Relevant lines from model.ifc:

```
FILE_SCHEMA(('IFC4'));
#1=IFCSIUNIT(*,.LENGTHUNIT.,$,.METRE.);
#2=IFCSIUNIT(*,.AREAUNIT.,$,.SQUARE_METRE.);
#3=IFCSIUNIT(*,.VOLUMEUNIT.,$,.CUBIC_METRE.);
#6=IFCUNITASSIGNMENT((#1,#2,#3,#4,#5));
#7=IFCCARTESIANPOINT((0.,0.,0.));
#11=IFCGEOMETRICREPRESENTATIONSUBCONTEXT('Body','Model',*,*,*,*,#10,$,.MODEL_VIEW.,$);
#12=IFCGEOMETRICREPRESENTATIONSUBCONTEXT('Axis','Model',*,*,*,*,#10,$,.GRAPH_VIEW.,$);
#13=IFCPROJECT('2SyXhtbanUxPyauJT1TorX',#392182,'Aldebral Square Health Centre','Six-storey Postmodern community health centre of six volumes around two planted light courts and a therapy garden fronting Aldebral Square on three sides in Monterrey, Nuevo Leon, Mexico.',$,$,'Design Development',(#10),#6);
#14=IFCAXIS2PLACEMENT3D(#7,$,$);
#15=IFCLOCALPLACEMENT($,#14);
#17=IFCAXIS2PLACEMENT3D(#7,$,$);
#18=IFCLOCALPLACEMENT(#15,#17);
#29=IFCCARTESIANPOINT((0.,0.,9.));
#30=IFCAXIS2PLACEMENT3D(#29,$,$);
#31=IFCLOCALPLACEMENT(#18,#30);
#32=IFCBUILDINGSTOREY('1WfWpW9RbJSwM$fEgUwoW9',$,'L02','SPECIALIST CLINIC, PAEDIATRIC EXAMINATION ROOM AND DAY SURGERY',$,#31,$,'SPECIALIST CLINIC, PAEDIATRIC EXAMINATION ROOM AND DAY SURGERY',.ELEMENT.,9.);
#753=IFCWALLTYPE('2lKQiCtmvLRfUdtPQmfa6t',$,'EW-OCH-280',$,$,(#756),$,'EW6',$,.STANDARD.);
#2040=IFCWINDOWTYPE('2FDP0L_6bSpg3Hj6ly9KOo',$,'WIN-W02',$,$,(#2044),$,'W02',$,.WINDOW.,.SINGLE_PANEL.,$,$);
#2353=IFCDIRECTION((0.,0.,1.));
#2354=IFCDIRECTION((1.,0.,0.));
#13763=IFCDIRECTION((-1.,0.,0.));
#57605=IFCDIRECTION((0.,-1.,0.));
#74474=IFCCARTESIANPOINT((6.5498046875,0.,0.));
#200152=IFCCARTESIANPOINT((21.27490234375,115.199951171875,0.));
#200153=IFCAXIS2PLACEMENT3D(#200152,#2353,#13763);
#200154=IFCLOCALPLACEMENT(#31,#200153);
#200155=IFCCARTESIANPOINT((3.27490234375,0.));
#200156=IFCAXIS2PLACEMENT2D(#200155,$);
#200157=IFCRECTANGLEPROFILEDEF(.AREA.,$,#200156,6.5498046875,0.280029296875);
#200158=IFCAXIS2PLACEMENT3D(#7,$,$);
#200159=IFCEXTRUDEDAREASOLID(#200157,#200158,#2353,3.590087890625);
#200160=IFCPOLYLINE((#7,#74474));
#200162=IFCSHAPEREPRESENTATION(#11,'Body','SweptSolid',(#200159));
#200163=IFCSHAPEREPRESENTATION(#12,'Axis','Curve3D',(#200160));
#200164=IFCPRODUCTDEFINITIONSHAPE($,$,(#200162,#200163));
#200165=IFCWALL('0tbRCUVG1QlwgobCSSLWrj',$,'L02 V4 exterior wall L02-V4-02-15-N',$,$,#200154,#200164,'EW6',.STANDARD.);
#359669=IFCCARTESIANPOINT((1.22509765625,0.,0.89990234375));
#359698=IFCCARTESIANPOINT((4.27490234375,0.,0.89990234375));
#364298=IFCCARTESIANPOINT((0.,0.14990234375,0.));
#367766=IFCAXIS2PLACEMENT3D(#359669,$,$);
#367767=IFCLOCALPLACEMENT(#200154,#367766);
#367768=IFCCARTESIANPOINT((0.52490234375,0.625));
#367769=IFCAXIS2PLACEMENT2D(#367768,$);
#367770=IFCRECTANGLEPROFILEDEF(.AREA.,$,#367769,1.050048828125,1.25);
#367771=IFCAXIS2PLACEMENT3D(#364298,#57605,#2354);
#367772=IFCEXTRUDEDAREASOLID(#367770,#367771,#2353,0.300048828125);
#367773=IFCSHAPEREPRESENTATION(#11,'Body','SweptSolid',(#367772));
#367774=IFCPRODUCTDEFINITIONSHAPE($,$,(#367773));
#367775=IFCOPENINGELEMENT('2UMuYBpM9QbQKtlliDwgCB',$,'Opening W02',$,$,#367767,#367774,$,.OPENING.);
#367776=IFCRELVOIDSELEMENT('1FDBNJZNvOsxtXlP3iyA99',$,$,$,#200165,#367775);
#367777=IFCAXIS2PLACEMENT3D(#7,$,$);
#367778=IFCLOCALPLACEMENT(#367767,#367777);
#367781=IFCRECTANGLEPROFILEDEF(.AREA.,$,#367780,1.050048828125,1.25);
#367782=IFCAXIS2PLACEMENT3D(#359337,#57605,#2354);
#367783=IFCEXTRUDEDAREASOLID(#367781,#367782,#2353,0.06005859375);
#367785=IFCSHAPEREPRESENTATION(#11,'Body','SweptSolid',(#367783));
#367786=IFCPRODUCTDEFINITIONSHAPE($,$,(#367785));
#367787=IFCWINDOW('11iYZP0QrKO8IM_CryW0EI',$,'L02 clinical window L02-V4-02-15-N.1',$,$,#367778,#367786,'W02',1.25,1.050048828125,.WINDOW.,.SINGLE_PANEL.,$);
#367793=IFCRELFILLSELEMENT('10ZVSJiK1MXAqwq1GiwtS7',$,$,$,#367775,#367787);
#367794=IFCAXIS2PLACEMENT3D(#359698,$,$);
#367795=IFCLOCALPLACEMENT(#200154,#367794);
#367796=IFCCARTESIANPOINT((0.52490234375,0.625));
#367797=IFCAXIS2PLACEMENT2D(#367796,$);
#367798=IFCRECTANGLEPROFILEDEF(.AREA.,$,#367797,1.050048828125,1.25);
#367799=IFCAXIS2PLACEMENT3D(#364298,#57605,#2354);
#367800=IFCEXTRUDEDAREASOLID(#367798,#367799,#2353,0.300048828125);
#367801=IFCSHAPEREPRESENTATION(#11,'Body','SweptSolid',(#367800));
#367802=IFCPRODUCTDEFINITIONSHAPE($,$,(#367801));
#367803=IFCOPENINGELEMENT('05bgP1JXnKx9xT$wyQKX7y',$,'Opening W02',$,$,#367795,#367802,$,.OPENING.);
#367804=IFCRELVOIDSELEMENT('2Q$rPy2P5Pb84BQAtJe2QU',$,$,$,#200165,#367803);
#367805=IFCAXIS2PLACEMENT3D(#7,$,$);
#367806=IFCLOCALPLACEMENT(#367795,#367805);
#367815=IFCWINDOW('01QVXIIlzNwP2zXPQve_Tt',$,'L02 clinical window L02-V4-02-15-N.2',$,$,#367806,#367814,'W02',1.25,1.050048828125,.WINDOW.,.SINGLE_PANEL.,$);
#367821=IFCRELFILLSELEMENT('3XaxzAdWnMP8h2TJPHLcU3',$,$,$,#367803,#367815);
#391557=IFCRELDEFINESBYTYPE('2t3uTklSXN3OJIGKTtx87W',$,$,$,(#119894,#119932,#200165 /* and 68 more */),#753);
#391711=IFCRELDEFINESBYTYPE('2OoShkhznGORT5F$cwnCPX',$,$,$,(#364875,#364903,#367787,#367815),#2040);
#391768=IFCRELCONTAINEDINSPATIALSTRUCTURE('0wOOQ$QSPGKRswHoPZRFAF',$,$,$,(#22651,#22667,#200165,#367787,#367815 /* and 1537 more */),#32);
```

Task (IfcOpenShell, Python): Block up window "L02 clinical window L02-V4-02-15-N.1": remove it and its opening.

```python
import ifcopenshell
import ifcopenshell.api.feature
import ifcopenshell.api.root
import ifcopenshell.geom
import ifcopenshell.util.shape

model = ifcopenshell.open("model.ifc")
settings = ifcopenshell.geom.settings()


def volume(element):
    """Net volume in cubic metres, openings subtracted."""
    shape = ifcopenshell.geom.create_shape(settings, element)
    return ifcopenshell.util.shape.get_volume(shape.geometry)


window = model.by_guid("11iYZP0QrKO8IM_CryW0EI")
opening = window.FillsVoids[0].RelatingOpeningElement
wall = opening.VoidsElements[0].RelatingBuildingElement
before = volume(wall)

ifcopenshell.api.root.remove_product(model, product=window)
ifcopenshell.api.feature.remove_feature(model, feature=opening)

after = volume(wall)

print(f"wall volume {before:.3f} -> {after:.3f} m3")

model.write("model_edited.ifc")
```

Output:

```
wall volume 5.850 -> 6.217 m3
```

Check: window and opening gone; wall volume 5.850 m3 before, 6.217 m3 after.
